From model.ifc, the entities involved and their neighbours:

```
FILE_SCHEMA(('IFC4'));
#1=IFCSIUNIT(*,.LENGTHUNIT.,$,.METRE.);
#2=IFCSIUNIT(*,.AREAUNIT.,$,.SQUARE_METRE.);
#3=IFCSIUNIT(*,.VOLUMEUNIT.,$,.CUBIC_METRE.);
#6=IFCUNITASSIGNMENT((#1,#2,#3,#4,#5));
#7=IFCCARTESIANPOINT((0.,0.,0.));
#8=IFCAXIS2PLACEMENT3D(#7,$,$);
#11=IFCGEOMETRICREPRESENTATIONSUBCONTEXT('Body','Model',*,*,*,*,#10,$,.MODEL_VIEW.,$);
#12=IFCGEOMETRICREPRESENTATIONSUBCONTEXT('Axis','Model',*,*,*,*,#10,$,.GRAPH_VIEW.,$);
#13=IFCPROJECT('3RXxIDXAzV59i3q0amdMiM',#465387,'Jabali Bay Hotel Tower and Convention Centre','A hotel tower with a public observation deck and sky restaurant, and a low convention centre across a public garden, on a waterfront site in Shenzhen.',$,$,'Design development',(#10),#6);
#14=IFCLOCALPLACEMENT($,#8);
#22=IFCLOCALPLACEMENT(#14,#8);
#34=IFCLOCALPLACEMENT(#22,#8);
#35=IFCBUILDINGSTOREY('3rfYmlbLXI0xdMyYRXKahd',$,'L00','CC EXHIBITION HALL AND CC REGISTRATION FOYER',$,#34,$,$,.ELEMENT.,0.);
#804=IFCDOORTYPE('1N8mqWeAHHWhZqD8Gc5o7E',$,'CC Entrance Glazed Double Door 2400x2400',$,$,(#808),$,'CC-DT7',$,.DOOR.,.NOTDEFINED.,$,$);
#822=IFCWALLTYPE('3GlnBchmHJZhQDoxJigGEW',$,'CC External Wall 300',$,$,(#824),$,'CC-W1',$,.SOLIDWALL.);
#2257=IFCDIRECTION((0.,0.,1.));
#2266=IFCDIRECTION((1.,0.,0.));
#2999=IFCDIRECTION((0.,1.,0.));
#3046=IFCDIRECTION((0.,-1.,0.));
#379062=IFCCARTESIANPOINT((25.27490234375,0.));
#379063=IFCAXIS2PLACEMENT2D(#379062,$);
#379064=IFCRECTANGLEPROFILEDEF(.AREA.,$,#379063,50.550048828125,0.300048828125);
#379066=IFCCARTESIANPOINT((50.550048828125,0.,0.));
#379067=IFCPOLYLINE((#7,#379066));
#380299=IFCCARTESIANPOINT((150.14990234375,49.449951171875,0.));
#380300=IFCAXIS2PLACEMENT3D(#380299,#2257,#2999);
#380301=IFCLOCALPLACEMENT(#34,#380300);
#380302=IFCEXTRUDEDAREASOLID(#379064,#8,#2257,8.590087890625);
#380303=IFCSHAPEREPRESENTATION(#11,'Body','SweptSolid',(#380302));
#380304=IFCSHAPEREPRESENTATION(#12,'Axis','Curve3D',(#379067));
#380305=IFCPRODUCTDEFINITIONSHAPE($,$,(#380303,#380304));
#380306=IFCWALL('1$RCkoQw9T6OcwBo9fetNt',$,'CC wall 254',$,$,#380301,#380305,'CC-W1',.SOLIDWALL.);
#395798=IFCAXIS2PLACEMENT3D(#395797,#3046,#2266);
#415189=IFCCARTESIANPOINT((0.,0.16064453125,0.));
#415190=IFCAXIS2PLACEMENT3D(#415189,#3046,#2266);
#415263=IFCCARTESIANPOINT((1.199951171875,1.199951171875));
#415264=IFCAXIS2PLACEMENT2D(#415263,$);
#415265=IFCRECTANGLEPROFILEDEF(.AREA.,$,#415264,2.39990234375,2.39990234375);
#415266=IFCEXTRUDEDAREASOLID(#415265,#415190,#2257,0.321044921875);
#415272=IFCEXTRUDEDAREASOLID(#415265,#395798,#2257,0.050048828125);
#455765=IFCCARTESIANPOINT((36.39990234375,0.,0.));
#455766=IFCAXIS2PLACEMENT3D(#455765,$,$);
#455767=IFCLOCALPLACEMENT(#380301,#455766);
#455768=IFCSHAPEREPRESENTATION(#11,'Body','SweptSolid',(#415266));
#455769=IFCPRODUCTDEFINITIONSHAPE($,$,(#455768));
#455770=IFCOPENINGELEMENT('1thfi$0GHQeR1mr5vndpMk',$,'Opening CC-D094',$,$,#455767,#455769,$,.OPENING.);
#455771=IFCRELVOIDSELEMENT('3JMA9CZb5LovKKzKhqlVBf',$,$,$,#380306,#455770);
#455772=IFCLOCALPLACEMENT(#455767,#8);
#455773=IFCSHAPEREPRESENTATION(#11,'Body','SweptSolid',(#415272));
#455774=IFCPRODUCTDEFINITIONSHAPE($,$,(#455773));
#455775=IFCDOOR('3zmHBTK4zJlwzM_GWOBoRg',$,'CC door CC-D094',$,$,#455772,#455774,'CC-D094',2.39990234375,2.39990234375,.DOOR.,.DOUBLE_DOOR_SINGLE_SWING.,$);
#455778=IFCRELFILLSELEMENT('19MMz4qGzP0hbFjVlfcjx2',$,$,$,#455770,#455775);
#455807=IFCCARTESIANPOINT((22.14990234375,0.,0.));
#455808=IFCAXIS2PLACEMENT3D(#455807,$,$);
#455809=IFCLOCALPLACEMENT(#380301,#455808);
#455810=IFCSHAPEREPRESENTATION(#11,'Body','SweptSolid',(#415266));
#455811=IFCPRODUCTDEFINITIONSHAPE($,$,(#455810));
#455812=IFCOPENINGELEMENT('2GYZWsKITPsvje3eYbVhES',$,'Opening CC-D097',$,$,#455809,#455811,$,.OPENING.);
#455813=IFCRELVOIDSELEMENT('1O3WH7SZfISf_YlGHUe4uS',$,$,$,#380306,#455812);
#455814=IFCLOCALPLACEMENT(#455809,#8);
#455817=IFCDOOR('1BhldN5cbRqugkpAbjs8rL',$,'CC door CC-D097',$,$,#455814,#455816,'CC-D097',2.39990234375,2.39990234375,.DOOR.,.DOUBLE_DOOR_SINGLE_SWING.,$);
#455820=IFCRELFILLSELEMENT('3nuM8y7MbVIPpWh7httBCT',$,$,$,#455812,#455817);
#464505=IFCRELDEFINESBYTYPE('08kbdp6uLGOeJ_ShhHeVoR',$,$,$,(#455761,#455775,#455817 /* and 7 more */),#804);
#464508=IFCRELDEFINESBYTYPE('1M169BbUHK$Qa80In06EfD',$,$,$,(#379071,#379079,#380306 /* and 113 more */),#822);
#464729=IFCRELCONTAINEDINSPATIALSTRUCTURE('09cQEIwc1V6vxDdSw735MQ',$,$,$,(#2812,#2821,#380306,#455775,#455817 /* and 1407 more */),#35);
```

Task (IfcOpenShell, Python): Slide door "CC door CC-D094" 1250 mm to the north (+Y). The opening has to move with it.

```python
import ifcopenshell
import ifcopenshell.api.geometry
import ifcopenshell.util.placement

model = ifcopenshell.open("model.ifc")

door = model.by_id(455775)
opening = door.FillsVoids[0].RelatingOpeningElement
wall = opening.VoidsElements[0].RelatingBuildingElement

wall_matrix = ifcopenshell.util.placement.get_local_placement(wall.ObjectPlacement)
shift = wall_matrix[:3, 0] * 1.25
before = ifcopenshell.util.placement.get_local_placement(door.ObjectPlacement)[:3, 3].copy()

# The door is placed relative to its opening, so it follows when the opening moves.
matrix = ifcopenshell.util.placement.get_local_placement(opening.ObjectPlacement)
matrix[:3, 3] += shift
ifcopenshell.api.geometry.edit_object_placement(
    model, product=opening, matrix=matrix, is_si=False, should_transform_children=True
)

after = ifcopenshell.util.placement.get_local_placement(door.ObjectPlacement)[:3, 3]
print("door moved by", (after - before).round(3) + 0.0)

model.write("model-out.ifc")
```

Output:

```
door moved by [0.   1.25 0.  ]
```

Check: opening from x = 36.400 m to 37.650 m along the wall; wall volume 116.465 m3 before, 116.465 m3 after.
